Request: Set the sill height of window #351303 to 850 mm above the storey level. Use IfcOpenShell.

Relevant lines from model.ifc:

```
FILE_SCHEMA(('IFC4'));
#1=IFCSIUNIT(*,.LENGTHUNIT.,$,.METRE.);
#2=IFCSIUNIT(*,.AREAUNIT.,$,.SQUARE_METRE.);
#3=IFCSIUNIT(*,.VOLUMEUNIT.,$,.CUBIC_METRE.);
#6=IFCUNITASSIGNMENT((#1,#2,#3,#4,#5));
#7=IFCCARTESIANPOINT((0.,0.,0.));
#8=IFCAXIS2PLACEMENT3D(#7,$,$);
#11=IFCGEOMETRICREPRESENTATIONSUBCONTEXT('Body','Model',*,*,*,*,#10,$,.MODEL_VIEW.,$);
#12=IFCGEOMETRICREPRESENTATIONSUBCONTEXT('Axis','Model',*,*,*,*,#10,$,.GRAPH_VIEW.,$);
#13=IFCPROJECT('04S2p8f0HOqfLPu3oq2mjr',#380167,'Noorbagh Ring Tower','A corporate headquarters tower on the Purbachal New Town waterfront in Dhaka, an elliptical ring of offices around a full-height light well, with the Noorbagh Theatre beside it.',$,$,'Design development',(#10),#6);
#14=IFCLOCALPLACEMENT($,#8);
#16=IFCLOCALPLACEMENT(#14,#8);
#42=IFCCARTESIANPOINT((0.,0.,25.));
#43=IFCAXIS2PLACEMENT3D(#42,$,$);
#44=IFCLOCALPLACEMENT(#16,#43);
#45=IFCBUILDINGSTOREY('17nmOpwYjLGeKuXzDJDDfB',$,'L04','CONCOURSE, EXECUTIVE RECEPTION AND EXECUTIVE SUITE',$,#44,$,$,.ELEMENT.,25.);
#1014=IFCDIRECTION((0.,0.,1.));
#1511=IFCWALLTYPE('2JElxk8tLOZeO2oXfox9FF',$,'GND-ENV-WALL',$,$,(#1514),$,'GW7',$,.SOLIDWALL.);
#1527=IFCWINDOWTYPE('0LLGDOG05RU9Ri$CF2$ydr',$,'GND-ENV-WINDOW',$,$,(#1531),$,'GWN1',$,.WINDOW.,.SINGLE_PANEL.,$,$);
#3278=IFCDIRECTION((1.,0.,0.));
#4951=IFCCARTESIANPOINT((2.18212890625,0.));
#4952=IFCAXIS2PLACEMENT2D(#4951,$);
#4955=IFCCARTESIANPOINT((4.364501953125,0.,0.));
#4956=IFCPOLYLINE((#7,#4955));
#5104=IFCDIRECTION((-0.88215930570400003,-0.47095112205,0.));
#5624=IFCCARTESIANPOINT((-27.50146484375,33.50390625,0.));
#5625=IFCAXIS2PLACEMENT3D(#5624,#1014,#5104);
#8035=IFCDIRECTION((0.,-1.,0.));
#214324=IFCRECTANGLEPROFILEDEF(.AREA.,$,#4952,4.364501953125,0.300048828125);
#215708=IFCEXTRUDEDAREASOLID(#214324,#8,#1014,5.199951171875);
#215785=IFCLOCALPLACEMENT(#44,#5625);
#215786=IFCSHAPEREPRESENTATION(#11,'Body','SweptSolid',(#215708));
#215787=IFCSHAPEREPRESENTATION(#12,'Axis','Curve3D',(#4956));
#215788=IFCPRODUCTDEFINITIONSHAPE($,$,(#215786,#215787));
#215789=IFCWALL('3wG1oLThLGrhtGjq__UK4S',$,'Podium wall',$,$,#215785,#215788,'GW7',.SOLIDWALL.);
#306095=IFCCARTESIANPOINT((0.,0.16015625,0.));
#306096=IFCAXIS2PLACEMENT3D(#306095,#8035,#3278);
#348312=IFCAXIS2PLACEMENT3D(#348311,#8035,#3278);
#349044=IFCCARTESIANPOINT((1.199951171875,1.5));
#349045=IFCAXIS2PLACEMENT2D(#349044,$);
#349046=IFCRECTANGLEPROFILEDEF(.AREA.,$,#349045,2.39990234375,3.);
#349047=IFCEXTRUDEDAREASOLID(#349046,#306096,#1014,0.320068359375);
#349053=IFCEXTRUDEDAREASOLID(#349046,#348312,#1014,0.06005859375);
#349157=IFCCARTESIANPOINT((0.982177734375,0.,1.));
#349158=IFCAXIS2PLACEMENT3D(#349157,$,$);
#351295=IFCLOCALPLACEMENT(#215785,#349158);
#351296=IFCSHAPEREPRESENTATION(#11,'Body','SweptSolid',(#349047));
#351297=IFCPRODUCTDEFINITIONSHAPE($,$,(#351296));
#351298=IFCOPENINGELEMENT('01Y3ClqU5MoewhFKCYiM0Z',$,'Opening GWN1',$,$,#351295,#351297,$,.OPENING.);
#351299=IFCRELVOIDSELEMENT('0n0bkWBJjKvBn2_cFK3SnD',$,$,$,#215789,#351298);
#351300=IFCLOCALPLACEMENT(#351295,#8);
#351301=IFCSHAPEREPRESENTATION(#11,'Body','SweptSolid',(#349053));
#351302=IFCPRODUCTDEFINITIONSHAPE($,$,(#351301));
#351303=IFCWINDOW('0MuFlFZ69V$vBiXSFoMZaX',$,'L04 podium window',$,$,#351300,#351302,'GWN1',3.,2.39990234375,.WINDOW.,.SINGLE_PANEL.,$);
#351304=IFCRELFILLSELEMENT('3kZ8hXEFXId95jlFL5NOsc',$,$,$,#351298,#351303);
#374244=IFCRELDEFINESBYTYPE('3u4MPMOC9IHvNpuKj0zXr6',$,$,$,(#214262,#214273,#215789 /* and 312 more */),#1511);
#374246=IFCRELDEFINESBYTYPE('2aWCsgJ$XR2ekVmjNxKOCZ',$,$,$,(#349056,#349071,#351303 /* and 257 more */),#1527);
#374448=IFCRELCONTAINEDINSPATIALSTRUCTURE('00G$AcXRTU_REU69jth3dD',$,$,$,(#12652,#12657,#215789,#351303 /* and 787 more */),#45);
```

```python
import numpy as np
import ifcopenshell
import ifcopenshell.api.geometry
import ifcopenshell.geom
import ifcopenshell.util.element
import ifcopenshell.util.placement
import ifcopenshell.util.shape
import ifcopenshell.util.unit

model = ifcopenshell.open("model.ifc")
unit_scale = ifcopenshell.util.unit.calculate_unit_scale(model)

window = model.by_guid("0MuFlFZ69V$vBiXSFoMZaX")
opening = window.FillsVoids[0].RelatingOpeningElement
storey = ifcopenshell.util.element.get_container(window, ifc_class="IfcBuildingStorey")
level = ifcopenshell.util.placement.get_local_placement(storey.ObjectPlacement)[2, 3]

# The opening's origin need not be at the sill, so measure its lowest point.
shape = ifcopenshell.geom.create_shape(ifcopenshell.geom.settings(), opening)
bottom = ifcopenshell.util.shape.get_shape_bottom_elevation(shape, shape.geometry) / unit_scale
dz = level + 0.85 / unit_scale - bottom

shift = np.array([0.0, 0.0, dz])
# The window is placed relative to its opening, so it follows when the opening moves.
matrix = ifcopenshell.util.placement.get_local_placement(opening.ObjectPlacement)
matrix[:3, 3] += shift
ifcopenshell.api.geometry.edit_object_placement(
    model, product=opening, matrix=matrix, is_si=False, should_transform_children=True
)

print(f"moved by {dz * unit_scale:+.3f} m")

model.write("model_updated.ifc")
```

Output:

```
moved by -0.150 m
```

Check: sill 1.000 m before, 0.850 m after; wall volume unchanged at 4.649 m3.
